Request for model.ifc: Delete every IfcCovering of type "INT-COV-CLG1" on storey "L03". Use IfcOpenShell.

First a look at what the model holds.

```python
import ifcopenshell
import ifcopenshell.util.element

model = ifcopenshell.open("model.ifc")
print(model.schema)
storey = next(s for s in model.by_type("IfcBuildingStorey") if s.Name == "L03")
coverings = [e for e in ifcopenshell.util.element.get_decomposition(storey) if e.is_a("IfcCovering")]
seen = {}
for e in coverings:
    element_type = ifcopenshell.util.element.get_type(e)
    name = element_type.Name if element_type not in (None, e) else None
    seen[name] = seen.get(name, 0) + 1
for name, count in sorted(seen.items(), key=str):
    print(count, "x", name)
```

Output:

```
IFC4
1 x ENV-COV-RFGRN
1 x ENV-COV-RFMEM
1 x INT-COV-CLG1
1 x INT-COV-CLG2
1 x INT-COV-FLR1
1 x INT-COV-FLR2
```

```python
import ifcopenshell
import ifcopenshell.api.root
import ifcopenshell.util.element

model = ifcopenshell.open("model.ifc")

storey = next(s for s in model.by_type("IfcBuildingStorey") if s.Name == "L03")
coverings = [e for e in ifcopenshell.util.element.get_decomposition(storey) if e.is_a("IfcCovering")]
targets = [e for e in coverings if (t := ifcopenshell.util.element.get_type(e)) not in (None, e) and t.Name == "INT-COV-CLG1"]

for e in targets:
    ifcopenshell.api.root.remove_product(model, product=e)
print(len(targets), "removed")

model.write("model_updated.ifc")
```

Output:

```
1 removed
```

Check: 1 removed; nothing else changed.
